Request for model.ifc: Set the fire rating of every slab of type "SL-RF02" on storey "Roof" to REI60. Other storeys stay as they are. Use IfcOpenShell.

First a look at what the model holds.

```python
import ifcopenshell
import ifcopenshell.util.element

model = ifcopenshell.open("model.ifc")
print(model.schema)
storey = next(s for s in model.by_type("IfcBuildingStorey") if s.Name == "Roof")
slabs = [e for e in ifcopenshell.util.element.get_decomposition(storey) if e.is_a("IfcSlab")]
seen = {}
for e in slabs:
    element_type = ifcopenshell.util.element.get_type(e)
    key = (element_type.Name if element_type != e and element_type else None, ifcopenshell.util.element.get_pset(e, "Pset_SlabCommon", "FireRating"))
    seen[key] = seen.get(key, 0) + 1
for (name, value), count in sorted(seen.items(), key=str):
    print(count, "x", name, "|", value)
```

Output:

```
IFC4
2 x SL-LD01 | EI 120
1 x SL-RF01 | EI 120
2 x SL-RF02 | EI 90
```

```python
import ifcopenshell
import ifcopenshell.api.pset
import ifcopenshell.util.element

model = ifcopenshell.open("model.ifc")

storey = next(s for s in model.by_type("IfcBuildingStorey") if s.Name == "Roof")
slabs = [e for e in ifcopenshell.util.element.get_decomposition(storey) if e.is_a("IfcSlab")]

count = 0
for e in slabs:
    element_type = ifcopenshell.util.element.get_type(e)
    if element_type in (None, e) or element_type.Name != "SL-RF02":
        continue
    # add_pset returns the element's existing set when there is one.
    pset = ifcopenshell.api.pset.add_pset(model, product=e, name="Pset_SlabCommon")
    ifcopenshell.api.pset.edit_pset(model, pset=pset, properties={"FireRating": "REI60"})
    count += 1

print(count, "slabs updated")

model.write("model-out.ifc")
```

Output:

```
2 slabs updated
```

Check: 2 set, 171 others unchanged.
